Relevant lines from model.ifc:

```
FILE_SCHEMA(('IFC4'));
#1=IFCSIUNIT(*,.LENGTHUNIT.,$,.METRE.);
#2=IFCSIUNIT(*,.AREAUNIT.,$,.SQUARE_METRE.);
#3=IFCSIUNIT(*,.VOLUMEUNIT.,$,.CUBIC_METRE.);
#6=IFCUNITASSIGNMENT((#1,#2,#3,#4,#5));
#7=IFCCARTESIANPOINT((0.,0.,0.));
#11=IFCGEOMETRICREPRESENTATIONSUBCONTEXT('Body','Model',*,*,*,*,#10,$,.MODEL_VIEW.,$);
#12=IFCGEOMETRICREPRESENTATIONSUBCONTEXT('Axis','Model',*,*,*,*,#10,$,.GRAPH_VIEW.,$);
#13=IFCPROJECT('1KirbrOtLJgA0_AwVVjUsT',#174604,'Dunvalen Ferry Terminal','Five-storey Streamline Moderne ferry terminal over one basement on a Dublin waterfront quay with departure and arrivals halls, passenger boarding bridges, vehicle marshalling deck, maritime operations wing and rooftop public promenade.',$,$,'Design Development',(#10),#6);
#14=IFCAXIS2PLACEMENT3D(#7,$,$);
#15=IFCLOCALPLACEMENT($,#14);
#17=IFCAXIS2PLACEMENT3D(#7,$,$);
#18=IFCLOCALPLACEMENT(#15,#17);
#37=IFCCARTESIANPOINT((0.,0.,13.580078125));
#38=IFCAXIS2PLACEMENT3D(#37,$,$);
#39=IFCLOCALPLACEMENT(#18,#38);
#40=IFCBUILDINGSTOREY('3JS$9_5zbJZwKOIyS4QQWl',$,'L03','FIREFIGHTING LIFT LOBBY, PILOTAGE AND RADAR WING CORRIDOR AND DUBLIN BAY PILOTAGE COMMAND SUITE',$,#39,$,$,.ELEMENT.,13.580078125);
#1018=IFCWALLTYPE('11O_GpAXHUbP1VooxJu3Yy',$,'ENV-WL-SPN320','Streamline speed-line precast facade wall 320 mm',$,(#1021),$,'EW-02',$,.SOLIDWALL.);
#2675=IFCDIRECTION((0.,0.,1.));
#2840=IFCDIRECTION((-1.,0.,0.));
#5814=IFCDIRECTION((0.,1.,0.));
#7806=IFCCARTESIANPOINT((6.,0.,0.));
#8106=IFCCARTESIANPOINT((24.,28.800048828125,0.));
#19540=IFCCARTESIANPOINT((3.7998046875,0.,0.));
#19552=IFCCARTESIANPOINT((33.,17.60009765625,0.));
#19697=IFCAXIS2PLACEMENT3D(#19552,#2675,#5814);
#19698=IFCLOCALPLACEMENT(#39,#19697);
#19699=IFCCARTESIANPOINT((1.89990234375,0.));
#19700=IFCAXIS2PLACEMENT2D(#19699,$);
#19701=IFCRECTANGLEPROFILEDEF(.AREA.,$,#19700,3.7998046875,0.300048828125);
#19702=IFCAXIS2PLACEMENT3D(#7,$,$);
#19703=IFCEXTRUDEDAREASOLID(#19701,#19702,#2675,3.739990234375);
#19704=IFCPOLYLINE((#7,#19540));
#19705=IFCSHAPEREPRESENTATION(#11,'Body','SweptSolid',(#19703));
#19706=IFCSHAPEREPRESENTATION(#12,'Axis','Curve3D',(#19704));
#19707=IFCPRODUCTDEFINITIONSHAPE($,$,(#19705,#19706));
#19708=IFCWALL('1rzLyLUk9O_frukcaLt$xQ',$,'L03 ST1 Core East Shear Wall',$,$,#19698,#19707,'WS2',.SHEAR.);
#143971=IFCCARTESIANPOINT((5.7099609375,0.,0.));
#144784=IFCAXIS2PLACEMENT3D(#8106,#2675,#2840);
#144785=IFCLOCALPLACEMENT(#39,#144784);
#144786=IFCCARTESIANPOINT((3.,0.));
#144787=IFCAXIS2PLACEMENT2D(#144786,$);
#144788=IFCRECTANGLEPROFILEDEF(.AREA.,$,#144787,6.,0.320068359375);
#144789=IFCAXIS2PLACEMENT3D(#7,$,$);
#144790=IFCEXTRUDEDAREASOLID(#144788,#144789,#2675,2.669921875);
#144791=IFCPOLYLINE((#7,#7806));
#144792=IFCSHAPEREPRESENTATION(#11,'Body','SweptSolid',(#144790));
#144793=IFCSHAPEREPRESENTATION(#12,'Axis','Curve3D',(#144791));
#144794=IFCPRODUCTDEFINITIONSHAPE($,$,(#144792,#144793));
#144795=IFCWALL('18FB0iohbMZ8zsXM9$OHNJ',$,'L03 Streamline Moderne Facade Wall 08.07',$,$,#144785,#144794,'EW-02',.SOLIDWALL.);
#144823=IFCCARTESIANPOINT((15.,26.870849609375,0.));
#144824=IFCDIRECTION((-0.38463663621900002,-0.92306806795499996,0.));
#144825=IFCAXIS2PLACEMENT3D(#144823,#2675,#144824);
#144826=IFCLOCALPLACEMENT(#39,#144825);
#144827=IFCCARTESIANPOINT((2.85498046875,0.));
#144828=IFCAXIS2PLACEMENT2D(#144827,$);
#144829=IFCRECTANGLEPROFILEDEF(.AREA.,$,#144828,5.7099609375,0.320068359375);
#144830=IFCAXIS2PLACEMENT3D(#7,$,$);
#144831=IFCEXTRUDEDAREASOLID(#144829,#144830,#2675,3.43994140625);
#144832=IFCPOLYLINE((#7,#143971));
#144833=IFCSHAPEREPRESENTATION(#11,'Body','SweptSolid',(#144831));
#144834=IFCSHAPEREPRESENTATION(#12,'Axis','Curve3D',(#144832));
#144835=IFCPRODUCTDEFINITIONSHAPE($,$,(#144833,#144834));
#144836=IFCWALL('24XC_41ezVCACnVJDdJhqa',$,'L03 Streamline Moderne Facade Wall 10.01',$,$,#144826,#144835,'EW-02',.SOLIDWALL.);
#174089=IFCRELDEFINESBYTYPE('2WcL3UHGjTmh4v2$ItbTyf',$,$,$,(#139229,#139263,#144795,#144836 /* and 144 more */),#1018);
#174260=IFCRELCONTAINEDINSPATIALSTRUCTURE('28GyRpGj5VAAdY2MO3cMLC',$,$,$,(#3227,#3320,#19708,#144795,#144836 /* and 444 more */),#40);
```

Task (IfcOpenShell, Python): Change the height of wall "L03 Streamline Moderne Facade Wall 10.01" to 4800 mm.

```python
import ifcopenshell
import ifcopenshell.geom
import ifcopenshell.util.representation
import ifcopenshell.util.shape
import ifcopenshell.util.unit

model = ifcopenshell.open("model.ifc")
unit_scale = ifcopenshell.util.unit.calculate_unit_scale(model)
settings = ifcopenshell.geom.settings()


def volume(element):
    """Net volume in cubic metres, openings subtracted."""
    shape = ifcopenshell.geom.create_shape(settings, element)
    return ifcopenshell.util.shape.get_volume(shape.geometry)


wall = model.by_id(144836)
before = volume(wall)

body = ifcopenshell.util.representation.get_representation(wall, "Model", "Body")
solid = body.Items[0]
old_height = solid.Depth
solid.Depth = 4.8 / unit_scale
after = volume(wall)

print(f"height {old_height:g} -> {solid.Depth:g}, volume {before:.3f} -> {after:.3f} m3")

model.write("model_edited.ifc")
```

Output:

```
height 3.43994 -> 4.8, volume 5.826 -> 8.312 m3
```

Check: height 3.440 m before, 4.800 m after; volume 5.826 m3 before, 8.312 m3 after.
